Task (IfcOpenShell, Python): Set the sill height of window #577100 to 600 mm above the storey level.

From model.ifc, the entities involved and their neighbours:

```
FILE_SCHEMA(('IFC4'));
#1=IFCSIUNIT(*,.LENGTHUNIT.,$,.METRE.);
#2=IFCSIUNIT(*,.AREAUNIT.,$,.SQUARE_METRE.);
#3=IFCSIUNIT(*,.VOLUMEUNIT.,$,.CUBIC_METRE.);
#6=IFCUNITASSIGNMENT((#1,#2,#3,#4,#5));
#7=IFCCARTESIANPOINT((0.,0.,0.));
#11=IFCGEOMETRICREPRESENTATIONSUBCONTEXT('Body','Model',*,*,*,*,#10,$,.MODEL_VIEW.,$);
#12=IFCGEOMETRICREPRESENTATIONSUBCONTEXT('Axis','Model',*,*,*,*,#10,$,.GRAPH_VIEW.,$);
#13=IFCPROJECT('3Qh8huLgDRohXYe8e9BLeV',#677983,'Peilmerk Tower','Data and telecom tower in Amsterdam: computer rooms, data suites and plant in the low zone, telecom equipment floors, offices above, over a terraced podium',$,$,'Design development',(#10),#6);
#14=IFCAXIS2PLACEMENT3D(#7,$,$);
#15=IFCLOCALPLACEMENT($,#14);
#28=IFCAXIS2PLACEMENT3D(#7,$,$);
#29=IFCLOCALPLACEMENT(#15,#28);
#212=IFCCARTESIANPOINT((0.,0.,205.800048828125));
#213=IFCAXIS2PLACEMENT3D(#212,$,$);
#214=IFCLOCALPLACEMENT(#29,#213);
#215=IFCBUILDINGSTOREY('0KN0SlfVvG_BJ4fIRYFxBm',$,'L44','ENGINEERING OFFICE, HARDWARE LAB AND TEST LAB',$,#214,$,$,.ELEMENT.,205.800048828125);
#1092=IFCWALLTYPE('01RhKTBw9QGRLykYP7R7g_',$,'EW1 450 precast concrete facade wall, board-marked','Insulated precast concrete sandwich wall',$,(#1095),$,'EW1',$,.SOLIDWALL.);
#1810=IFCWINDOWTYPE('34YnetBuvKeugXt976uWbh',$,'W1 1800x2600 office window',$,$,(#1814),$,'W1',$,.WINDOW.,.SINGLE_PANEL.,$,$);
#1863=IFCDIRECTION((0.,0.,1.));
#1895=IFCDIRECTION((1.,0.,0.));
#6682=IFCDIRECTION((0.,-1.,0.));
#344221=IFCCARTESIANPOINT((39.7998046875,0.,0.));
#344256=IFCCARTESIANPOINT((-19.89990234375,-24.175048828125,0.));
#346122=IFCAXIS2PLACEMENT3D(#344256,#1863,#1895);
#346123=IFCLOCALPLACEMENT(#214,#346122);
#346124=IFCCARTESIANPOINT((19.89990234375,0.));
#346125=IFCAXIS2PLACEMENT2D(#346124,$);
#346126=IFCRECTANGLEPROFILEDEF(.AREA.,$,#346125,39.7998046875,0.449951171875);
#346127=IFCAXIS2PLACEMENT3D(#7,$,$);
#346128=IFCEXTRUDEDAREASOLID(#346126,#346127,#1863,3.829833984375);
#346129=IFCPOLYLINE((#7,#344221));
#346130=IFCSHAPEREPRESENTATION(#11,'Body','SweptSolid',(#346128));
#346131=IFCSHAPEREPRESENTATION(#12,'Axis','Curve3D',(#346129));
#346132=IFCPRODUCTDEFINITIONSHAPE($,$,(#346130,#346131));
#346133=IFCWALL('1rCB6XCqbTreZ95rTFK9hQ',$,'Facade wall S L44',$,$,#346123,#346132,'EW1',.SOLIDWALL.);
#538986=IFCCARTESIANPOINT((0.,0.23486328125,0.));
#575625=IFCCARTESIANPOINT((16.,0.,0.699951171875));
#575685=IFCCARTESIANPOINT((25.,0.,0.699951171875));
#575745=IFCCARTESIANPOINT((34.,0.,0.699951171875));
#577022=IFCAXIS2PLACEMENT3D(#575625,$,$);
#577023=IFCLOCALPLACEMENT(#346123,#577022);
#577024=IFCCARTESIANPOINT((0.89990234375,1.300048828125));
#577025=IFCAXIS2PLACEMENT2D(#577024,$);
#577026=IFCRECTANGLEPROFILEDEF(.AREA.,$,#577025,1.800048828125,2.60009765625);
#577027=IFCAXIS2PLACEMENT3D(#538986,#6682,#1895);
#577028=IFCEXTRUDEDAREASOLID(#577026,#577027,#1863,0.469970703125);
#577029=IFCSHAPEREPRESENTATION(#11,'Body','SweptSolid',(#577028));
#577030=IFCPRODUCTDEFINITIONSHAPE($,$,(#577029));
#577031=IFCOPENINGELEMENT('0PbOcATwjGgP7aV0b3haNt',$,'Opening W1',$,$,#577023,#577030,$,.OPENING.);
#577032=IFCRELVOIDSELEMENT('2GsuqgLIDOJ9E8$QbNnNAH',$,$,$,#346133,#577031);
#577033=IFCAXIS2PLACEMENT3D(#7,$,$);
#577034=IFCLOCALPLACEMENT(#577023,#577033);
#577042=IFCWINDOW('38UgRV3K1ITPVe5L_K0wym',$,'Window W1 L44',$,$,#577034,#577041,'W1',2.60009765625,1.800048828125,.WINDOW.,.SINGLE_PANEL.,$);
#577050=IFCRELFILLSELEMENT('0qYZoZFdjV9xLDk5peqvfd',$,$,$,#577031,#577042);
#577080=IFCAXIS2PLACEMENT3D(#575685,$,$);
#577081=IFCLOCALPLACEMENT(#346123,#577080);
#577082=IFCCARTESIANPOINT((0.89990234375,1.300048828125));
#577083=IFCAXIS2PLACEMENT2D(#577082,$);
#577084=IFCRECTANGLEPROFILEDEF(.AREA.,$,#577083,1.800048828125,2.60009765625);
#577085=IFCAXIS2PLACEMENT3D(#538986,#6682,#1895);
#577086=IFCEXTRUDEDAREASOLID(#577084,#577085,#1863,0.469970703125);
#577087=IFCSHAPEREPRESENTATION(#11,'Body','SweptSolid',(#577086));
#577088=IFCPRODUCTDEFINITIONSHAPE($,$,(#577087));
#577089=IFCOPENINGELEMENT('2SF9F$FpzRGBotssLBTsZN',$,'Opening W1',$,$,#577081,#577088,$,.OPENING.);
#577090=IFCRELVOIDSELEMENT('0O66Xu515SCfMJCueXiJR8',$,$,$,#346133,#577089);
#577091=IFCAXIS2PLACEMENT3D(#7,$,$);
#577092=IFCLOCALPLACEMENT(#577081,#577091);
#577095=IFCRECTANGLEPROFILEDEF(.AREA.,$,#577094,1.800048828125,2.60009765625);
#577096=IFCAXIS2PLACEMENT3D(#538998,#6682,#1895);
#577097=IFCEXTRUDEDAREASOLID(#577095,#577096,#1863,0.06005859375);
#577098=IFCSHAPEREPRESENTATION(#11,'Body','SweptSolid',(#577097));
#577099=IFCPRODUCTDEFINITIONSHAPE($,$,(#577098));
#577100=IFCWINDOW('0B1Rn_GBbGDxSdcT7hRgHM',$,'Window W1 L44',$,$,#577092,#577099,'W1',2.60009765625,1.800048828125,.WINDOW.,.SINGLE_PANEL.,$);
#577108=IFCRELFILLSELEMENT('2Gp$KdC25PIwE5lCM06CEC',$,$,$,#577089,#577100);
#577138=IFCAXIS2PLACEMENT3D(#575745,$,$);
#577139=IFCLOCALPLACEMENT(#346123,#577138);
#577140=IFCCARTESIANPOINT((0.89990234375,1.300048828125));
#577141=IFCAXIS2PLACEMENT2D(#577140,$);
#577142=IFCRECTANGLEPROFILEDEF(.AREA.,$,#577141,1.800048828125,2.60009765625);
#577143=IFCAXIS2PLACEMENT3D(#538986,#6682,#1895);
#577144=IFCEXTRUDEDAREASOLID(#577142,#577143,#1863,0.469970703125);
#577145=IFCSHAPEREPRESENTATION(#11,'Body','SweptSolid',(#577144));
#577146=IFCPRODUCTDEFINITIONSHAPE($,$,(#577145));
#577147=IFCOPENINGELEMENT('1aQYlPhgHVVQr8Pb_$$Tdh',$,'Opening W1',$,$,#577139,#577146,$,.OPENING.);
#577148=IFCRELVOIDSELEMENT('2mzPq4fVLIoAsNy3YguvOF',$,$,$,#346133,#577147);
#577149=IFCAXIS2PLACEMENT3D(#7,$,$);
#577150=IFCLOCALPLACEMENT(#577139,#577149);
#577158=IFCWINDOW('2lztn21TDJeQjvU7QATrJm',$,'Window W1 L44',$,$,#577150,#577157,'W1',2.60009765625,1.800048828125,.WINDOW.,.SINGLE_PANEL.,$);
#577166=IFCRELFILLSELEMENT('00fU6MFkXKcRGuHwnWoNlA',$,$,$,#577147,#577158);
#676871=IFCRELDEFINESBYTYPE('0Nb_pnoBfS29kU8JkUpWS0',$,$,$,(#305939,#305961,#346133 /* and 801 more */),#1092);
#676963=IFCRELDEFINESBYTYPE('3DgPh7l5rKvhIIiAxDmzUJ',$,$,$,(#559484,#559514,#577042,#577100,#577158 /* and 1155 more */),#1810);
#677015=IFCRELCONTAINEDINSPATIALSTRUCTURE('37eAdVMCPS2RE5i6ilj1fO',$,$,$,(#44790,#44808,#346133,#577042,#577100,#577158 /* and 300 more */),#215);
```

```python
import numpy as np
import ifcopenshell
import ifcopenshell.api.geometry
import ifcopenshell.geom
import ifcopenshell.util.element
import ifcopenshell.util.placement
import ifcopenshell.util.shape
import ifcopenshell.util.unit

model = ifcopenshell.open("model.ifc")
unit_scale = ifcopenshell.util.unit.calculate_unit_scale(model)

window = model.by_guid("0B1Rn_GBbGDxSdcT7hRgHM")
opening = window.FillsVoids[0].RelatingOpeningElement
storey = ifcopenshell.util.element.get_container(window, ifc_class="IfcBuildingStorey")
level = ifcopenshell.util.placement.get_local_placement(storey.ObjectPlacement)[2, 3]

# The opening's origin need not be at the sill, so measure its lowest point.
shape = ifcopenshell.geom.create_shape(ifcopenshell.geom.settings(), opening)
bottom = ifcopenshell.util.shape.get_shape_bottom_elevation(shape, shape.geometry) / unit_scale
dz = level + 0.6 / unit_scale - bottom

shift = np.array([0.0, 0.0, dz])
# The window is placed relative to its opening, so it follows when the opening moves.
matrix = ifcopenshell.util.placement.get_local_placement(opening.ObjectPlacement)
matrix[:3, 3] += shift
ifcopenshell.api.geometry.edit_object_placement(
    model, product=opening, matrix=matrix, is_si=False, should_transform_children=True
)

print(f"moved by {dz * unit_scale:+.3f} m")

model.write("model-out.ifc")
```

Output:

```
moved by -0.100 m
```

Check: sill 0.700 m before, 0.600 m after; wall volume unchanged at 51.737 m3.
